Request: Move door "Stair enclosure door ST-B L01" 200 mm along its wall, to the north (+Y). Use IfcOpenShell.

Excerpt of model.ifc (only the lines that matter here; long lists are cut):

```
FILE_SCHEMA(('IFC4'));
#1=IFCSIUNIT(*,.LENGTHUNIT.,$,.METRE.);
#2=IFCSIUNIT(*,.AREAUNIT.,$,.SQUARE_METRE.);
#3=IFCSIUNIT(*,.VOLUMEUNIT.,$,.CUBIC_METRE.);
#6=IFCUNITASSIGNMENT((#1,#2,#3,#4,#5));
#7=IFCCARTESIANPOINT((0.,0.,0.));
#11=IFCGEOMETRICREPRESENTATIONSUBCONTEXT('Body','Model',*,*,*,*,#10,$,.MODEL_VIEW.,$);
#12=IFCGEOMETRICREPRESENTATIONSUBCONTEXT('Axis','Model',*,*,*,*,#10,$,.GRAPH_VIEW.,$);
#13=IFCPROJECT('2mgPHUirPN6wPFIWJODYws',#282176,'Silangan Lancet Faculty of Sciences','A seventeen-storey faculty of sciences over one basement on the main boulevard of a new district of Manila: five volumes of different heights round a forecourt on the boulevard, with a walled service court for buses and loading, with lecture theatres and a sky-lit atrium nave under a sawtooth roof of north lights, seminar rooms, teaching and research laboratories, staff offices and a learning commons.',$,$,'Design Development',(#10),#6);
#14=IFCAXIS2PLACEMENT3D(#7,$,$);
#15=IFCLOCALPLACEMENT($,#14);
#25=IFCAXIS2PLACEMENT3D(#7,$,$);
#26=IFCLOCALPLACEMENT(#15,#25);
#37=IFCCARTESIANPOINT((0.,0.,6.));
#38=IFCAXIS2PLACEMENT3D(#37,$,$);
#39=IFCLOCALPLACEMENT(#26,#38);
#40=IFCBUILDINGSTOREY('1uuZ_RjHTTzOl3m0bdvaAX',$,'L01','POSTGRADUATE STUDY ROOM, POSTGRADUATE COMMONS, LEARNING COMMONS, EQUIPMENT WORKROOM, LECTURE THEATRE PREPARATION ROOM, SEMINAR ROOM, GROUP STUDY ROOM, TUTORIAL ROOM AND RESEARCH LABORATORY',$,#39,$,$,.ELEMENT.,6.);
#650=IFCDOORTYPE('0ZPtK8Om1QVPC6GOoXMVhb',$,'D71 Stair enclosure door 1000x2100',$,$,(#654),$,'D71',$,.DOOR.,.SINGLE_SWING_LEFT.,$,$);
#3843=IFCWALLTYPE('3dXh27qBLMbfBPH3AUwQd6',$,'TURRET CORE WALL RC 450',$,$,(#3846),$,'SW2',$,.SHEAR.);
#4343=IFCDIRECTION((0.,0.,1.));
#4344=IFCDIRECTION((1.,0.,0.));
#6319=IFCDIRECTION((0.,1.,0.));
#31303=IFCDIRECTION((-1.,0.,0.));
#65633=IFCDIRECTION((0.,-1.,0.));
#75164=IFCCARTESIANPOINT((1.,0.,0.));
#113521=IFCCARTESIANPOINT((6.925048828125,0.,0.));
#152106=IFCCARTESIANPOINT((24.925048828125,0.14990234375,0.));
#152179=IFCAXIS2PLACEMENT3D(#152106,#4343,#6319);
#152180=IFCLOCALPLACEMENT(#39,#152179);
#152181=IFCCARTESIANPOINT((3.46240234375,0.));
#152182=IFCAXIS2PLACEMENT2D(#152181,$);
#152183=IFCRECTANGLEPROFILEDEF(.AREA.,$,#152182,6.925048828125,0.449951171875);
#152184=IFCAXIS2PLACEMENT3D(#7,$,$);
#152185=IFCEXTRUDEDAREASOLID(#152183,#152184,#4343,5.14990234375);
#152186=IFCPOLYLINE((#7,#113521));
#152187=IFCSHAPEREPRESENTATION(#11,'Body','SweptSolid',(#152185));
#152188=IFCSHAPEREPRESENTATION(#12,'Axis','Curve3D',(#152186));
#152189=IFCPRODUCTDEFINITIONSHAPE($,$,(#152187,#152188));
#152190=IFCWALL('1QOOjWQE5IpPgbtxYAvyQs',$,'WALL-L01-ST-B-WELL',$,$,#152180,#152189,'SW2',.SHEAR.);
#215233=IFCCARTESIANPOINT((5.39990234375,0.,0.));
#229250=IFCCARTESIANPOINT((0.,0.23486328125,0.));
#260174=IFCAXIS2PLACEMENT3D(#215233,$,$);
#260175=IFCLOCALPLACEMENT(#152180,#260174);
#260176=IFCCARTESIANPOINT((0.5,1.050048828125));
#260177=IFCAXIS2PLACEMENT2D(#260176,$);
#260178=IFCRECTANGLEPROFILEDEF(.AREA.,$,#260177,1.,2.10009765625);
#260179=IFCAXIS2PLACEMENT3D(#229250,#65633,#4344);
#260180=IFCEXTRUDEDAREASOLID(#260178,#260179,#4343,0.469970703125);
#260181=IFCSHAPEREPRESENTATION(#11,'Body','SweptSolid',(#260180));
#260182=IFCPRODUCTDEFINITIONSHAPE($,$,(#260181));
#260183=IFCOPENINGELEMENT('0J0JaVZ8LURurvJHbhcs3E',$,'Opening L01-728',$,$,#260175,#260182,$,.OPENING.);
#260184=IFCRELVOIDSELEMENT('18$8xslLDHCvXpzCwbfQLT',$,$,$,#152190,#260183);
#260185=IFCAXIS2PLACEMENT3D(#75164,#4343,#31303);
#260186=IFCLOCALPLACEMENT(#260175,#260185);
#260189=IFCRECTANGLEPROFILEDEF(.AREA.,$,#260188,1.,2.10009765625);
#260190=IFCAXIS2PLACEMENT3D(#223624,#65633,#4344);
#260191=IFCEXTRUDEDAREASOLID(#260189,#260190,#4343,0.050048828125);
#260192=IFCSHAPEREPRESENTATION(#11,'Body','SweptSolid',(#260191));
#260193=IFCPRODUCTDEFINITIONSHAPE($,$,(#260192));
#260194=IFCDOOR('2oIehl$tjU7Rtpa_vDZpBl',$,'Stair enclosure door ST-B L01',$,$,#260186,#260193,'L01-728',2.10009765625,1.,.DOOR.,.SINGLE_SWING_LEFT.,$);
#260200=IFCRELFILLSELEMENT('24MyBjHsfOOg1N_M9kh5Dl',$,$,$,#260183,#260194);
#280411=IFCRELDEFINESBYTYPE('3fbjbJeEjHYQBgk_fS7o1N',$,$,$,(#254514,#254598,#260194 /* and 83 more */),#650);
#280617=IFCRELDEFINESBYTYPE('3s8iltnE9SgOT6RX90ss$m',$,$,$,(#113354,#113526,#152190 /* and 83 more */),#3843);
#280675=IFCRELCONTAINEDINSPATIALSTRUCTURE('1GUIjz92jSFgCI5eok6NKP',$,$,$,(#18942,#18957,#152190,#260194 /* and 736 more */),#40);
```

```python
import ifcopenshell
import ifcopenshell.api.geometry
import ifcopenshell.util.placement
import ifcopenshell.util.unit

model = ifcopenshell.open("model.ifc")
unit_scale = ifcopenshell.util.unit.calculate_unit_scale(model)

door = model.by_id(260194)
opening = door.FillsVoids[0].RelatingOpeningElement
wall = opening.VoidsElements[0].RelatingBuildingElement

wall_matrix = ifcopenshell.util.placement.get_local_placement(wall.ObjectPlacement)
shift = wall_matrix[:3, 0] * 0.2 / unit_scale
before = ifcopenshell.util.placement.get_local_placement(door.ObjectPlacement)[:3, 3].copy()

# The door is placed relative to its opening, so it follows when the opening moves.
matrix = ifcopenshell.util.placement.get_local_placement(opening.ObjectPlacement)
matrix[:3, 3] += shift
ifcopenshell.api.geometry.edit_object_placement(
    model, product=opening, matrix=matrix, is_si=False, should_transform_children=True
)

after = ifcopenshell.util.placement.get_local_placement(door.ObjectPlacement)[:3, 3]
print("door moved by", (after - before).round(3) + 0.0)

model.write("model_rev.ifc")
```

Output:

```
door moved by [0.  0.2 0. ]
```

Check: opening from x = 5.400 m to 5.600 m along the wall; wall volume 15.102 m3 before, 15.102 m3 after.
